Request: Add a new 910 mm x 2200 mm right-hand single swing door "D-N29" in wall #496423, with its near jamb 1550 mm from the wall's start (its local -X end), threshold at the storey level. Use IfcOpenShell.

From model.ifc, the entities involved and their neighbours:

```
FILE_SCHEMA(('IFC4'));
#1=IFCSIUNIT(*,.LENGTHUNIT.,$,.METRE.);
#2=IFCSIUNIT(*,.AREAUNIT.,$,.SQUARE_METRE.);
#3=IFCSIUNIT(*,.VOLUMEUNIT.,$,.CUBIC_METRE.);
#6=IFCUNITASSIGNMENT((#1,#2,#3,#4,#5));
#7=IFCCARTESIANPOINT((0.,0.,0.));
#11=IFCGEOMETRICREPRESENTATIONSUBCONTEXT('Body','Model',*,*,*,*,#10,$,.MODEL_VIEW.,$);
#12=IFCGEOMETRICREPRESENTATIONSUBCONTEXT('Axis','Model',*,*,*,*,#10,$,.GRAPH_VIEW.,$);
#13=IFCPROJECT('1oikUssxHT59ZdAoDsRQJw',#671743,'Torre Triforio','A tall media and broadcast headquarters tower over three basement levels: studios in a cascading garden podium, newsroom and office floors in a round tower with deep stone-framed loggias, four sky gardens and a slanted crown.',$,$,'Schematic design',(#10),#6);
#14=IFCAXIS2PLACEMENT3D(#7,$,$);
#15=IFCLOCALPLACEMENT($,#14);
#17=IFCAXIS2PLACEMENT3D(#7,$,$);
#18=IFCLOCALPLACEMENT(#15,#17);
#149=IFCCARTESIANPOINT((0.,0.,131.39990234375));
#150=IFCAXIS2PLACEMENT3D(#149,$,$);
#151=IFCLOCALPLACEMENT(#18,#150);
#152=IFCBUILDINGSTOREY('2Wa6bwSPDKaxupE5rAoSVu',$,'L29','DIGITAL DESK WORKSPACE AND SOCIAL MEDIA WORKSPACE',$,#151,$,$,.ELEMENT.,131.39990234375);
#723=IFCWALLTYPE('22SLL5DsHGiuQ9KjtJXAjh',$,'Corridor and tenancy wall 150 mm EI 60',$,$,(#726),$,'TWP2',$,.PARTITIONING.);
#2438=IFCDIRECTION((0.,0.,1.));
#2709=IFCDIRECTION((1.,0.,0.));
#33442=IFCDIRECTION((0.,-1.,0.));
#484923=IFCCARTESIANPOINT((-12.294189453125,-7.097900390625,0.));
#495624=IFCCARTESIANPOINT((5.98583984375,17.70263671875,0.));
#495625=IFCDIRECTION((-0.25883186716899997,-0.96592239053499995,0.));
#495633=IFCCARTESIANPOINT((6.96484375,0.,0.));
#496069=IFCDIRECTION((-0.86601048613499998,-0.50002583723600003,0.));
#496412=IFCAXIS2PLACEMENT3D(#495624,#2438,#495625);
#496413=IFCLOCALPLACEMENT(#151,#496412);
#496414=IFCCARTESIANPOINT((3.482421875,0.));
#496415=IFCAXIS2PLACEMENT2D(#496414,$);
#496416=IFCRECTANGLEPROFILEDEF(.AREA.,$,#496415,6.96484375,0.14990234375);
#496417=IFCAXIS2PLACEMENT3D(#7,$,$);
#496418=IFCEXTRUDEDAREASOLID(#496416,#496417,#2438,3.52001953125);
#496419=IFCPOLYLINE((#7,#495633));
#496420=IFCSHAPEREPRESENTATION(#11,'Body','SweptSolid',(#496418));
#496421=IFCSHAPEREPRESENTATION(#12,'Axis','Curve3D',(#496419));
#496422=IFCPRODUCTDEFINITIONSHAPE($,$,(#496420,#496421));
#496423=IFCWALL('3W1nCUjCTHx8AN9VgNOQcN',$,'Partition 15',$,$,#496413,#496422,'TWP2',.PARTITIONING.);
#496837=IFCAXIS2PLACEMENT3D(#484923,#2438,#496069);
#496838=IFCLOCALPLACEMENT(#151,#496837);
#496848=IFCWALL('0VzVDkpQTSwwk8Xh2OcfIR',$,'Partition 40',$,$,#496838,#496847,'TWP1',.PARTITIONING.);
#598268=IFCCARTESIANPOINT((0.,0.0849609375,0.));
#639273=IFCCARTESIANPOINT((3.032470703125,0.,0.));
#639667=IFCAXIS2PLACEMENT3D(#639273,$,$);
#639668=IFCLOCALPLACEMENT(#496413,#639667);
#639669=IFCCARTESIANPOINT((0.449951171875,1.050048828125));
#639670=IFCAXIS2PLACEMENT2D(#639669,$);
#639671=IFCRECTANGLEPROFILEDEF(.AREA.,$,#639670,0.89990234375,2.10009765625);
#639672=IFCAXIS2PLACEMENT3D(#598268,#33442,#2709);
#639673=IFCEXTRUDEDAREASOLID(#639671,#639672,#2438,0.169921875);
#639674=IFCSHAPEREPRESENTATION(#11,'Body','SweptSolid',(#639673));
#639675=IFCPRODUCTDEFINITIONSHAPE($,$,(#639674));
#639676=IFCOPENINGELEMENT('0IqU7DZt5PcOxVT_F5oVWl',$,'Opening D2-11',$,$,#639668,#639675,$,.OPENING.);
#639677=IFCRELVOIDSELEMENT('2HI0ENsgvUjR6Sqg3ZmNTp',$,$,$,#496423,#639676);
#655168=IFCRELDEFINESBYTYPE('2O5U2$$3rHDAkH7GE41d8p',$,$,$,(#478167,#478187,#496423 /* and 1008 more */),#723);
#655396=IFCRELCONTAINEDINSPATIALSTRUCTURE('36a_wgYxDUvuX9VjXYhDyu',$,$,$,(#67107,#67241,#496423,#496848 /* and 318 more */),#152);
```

```python
import numpy as np
import ifcopenshell
import ifcopenshell.api.feature
import ifcopenshell.api.geometry
import ifcopenshell.api.root
import ifcopenshell.api.spatial
import ifcopenshell.geom
import ifcopenshell.util.element
import ifcopenshell.util.placement
import ifcopenshell.util.representation
import ifcopenshell.util.shape
import ifcopenshell.util.unit

model = ifcopenshell.open("model.ifc")
unit_scale = ifcopenshell.util.unit.calculate_unit_scale(model)
settings = ifcopenshell.geom.settings()


def volume(element):
    """Net volume in cubic metres, openings subtracted."""
    shape = ifcopenshell.geom.create_shape(settings, element)
    return ifcopenshell.util.shape.get_volume(shape.geometry)


wall = model.by_id(496423)
storey = ifcopenshell.util.element.get_container(wall, ifc_class="IfcBuildingStorey")
context = ifcopenshell.util.representation.get_context(model, "Model", "Body", "MODEL_VIEW")
before = volume(wall)

width, height, from_end, sill = 0.91, 2.2, 1.55, 0.0  # metres

# The wall runs along its own X axis, and the end named is its -X end.
wall_shape = ifcopenshell.geom.create_shape(settings, wall)
x, y, z = ifcopenshell.util.shape.get_vertices(wall_shape.geometry).T
start = x.min() + from_end
face, thickness = float(y.min()), float(y.max() - y.min())
wall_matrix = ifcopenshell.util.placement.get_local_placement(wall.ObjectPlacement)
level = ifcopenshell.util.placement.get_local_placement(storey.ObjectPlacement)[2, 3]


def in_wall(x, y):
    """Placement at x, y metres in the wall's axes, at sill height."""
    matrix = wall_matrix.copy()
    matrix[:, 3] = wall_matrix @ np.array([x / unit_scale, y / unit_scale, 0.0, 1.0])
    matrix[2, 3] = level + sill / unit_scale
    return matrix


# Opening: a box that overshoots both wall faces by 50 mm.
opening = ifcopenshell.api.root.create_entity(model, ifc_class="IfcOpeningElement", predefined_type="OPENING")
box = ifcopenshell.api.geometry.add_wall_representation(
    model, context=context, length=width, height=height, thickness=thickness + 0.1
)
ifcopenshell.api.geometry.assign_representation(model, product=opening, representation=box)
ifcopenshell.api.geometry.edit_object_placement(model, product=opening, matrix=in_wall(start, face - 0.05), is_si=False)
ifcopenshell.api.feature.add_feature(model, feature=opening, element=wall)

door = ifcopenshell.api.root.create_entity(model, ifc_class="IfcDoor", name="D-N29", predefined_type="DOOR")
door.OverallWidth, door.OverallHeight = width / unit_scale, height / unit_scale
door.OperationType = "SINGLE_SWING_RIGHT"
body = ifcopenshell.api.geometry.add_door_representation(
    model,
    context=context,
    overall_width=door.OverallWidth,
    overall_height=door.OverallHeight,
    operation_type="SINGLE_SWING_RIGHT",
    lining_properties={"LiningDepth": thickness / unit_scale, "ThresholdDepth": thickness / unit_scale},
)
ifcopenshell.api.geometry.assign_representation(model, product=door, representation=body)
ifcopenshell.api.spatial.assign_container(model, products=[door], relating_structure=storey)
ifcopenshell.api.feature.add_filling(model, opening=opening, element=door)

# The lining spans the wall, so the door starts at the wall face.
ifcopenshell.api.geometry.edit_object_placement(model, product=door, matrix=in_wall(start, face), is_si=False)

after = volume(wall)

print(f"wall volume {before:.3f} -> {after:.3f} m3")

model.write("model_updated.ifc")
```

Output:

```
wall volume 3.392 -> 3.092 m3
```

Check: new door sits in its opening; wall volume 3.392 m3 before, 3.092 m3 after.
